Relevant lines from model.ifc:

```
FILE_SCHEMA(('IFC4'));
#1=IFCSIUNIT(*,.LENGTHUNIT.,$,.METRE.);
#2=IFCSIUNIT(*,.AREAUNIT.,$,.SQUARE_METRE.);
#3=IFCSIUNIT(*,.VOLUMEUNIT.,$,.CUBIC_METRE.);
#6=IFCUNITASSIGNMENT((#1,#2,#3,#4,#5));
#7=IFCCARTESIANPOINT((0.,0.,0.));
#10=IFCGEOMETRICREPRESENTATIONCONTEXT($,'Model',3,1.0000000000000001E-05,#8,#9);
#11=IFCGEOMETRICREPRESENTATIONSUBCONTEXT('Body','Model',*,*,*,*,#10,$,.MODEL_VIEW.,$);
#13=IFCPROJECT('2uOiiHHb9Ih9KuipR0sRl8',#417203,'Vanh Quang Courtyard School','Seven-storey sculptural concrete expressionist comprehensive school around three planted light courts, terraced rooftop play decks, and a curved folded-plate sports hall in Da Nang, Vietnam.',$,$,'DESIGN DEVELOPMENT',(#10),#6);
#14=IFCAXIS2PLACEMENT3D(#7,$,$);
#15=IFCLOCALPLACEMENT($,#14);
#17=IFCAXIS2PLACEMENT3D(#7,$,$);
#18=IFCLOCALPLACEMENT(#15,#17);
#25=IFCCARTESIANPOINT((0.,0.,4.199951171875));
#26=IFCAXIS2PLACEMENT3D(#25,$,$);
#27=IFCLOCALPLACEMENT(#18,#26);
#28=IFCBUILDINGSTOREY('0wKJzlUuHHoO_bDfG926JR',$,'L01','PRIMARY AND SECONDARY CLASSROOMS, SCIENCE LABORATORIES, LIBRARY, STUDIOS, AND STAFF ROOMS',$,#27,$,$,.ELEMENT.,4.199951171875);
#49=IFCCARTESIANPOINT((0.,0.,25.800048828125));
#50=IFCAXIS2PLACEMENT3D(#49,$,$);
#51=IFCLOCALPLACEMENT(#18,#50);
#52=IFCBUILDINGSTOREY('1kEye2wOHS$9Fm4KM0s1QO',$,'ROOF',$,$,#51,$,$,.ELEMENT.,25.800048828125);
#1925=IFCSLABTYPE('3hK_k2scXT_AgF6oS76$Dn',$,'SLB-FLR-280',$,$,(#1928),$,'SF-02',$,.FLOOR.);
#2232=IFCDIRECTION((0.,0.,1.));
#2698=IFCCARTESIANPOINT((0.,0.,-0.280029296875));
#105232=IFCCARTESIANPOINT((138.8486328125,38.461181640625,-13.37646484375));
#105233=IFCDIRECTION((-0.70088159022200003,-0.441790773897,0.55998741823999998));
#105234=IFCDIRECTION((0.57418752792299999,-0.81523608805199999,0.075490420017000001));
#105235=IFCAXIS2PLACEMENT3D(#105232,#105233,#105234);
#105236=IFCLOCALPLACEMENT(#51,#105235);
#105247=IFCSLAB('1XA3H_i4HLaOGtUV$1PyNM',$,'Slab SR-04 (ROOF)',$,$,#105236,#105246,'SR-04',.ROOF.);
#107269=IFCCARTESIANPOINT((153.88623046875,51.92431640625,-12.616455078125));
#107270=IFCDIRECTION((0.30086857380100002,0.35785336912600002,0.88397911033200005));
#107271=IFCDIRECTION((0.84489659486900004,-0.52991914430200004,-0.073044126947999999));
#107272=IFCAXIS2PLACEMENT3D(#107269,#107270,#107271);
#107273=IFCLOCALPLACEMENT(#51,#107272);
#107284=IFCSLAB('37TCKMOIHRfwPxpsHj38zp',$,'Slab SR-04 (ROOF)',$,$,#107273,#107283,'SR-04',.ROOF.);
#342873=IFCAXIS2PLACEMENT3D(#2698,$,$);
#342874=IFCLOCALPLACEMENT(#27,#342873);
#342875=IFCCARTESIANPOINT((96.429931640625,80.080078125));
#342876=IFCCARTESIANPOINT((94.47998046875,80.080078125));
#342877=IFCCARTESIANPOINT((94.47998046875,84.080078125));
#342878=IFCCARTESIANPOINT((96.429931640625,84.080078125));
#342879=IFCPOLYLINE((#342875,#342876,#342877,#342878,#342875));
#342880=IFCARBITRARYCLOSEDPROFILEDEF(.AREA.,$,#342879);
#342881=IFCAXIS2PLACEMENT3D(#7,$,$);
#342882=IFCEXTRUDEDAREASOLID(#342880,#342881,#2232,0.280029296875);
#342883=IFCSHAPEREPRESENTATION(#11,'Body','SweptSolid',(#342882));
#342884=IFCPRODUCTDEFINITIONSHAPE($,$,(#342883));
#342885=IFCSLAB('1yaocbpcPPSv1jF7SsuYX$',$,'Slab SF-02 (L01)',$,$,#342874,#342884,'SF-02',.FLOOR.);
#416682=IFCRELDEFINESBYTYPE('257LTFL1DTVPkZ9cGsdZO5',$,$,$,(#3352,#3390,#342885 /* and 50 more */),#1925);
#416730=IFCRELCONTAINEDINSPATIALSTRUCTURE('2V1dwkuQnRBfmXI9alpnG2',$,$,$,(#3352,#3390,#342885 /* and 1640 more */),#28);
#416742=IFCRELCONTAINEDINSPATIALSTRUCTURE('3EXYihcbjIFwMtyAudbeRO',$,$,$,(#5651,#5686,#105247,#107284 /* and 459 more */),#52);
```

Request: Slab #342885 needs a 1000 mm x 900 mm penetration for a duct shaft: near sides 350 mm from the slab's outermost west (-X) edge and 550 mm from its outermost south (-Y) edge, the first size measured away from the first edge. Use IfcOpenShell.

```python
import numpy as np
import ifcopenshell
import ifcopenshell.api.feature
import ifcopenshell.api.geometry
import ifcopenshell.api.root
import ifcopenshell.geom
import ifcopenshell.util.placement
import ifcopenshell.util.representation
import ifcopenshell.util.shape
import ifcopenshell.util.unit

model = ifcopenshell.open("model.ifc")
unit_scale = ifcopenshell.util.unit.calculate_unit_scale(model)
settings = ifcopenshell.geom.settings()


def volume(element):
    """Net volume in cubic metres, openings subtracted."""
    shape = ifcopenshell.geom.create_shape(settings, element)
    return ifcopenshell.util.shape.get_volume(shape.geometry)


slab = model.by_guid("1yaocbpcPPSv1jF7SsuYX$")
before = volume(slab)

# Extent in the slab's own axes, in metres. The edges named are its -X and -Y sides.
slab_shape = ifcopenshell.geom.create_shape(settings, slab)
vertices = ifcopenshell.util.shape.get_vertices(slab_shape.geometry)
x_min, y_min, bottom = vertices.min(axis=0)
top = vertices[:, 2].max()

opening = ifcopenshell.api.root.create_entity(model, ifc_class="IfcOpeningElement", name="Duct shaft opening", predefined_type="OPENING")
context = ifcopenshell.util.representation.get_context(model, "Model", "Body", "MODEL_VIEW")
width, depth = 1, 0.9
outline = [(0.0, 0.0), (width, 0.0), (width, depth), (0.0, depth), (0.0, 0.0)]
# Overshoot both faces by 50 mm so the cut is clean.
shape = ifcopenshell.api.geometry.add_slab_representation(
    model, context=context, depth=top - bottom + 0.1, polyline=outline
)
ifcopenshell.api.geometry.assign_representation(model, product=opening, representation=shape)

matrix = ifcopenshell.util.placement.get_local_placement(slab.ObjectPlacement)
matrix[:, 3] = matrix @ np.append(np.array([x_min + 0.35, y_min + 0.55, bottom - 0.05]) / unit_scale, 1.0)
ifcopenshell.api.geometry.edit_object_placement(model, product=opening, matrix=matrix, is_si=False)
ifcopenshell.api.feature.add_feature(model, feature=opening, element=slab)

after = volume(slab)

print(f"slab volume {before:.3f} -> {after:.3f} m3")

model.write("model_edited.ifc")
```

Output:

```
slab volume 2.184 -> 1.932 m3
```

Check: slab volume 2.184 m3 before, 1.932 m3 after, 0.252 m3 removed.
